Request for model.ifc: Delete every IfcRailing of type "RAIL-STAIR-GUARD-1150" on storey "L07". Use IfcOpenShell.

First a look at what the model holds.

```python
import ifcopenshell
import ifcopenshell.util.element

model = ifcopenshell.open("model.ifc")
print(model.schema)
storey = next(s for s in model.by_type("IfcBuildingStorey") if s.Name == "L07")
railings = [e for e in ifcopenshell.util.element.get_decomposition(storey) if e.is_a("IfcRailing")]
seen = {}
for e in railings:
    element_type = ifcopenshell.util.element.get_type(e)
    name = element_type.Name if element_type not in (None, e) else None
    seen[name] = seen.get(name, 0) + 1
for name, count in sorted(seen.items(), key=str):
    print(count, "x", name)
```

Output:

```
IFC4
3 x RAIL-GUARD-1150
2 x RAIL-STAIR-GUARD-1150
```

```python
import ifcopenshell
import ifcopenshell.api.root
import ifcopenshell.util.element

model = ifcopenshell.open("model.ifc")

storey = next(s for s in model.by_type("IfcBuildingStorey") if s.Name == "L07")
railings = [e for e in ifcopenshell.util.element.get_decomposition(storey) if e.is_a("IfcRailing")]
targets = [e for e in railings if (t := ifcopenshell.util.element.get_type(e)) not in (None, e) and t.Name == "RAIL-STAIR-GUARD-1150"]

for e in targets:
    ifcopenshell.api.root.remove_product(model, product=e)
print(len(targets), "removed")

model.write("model-out.ifc")
```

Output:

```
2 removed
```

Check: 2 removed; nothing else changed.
